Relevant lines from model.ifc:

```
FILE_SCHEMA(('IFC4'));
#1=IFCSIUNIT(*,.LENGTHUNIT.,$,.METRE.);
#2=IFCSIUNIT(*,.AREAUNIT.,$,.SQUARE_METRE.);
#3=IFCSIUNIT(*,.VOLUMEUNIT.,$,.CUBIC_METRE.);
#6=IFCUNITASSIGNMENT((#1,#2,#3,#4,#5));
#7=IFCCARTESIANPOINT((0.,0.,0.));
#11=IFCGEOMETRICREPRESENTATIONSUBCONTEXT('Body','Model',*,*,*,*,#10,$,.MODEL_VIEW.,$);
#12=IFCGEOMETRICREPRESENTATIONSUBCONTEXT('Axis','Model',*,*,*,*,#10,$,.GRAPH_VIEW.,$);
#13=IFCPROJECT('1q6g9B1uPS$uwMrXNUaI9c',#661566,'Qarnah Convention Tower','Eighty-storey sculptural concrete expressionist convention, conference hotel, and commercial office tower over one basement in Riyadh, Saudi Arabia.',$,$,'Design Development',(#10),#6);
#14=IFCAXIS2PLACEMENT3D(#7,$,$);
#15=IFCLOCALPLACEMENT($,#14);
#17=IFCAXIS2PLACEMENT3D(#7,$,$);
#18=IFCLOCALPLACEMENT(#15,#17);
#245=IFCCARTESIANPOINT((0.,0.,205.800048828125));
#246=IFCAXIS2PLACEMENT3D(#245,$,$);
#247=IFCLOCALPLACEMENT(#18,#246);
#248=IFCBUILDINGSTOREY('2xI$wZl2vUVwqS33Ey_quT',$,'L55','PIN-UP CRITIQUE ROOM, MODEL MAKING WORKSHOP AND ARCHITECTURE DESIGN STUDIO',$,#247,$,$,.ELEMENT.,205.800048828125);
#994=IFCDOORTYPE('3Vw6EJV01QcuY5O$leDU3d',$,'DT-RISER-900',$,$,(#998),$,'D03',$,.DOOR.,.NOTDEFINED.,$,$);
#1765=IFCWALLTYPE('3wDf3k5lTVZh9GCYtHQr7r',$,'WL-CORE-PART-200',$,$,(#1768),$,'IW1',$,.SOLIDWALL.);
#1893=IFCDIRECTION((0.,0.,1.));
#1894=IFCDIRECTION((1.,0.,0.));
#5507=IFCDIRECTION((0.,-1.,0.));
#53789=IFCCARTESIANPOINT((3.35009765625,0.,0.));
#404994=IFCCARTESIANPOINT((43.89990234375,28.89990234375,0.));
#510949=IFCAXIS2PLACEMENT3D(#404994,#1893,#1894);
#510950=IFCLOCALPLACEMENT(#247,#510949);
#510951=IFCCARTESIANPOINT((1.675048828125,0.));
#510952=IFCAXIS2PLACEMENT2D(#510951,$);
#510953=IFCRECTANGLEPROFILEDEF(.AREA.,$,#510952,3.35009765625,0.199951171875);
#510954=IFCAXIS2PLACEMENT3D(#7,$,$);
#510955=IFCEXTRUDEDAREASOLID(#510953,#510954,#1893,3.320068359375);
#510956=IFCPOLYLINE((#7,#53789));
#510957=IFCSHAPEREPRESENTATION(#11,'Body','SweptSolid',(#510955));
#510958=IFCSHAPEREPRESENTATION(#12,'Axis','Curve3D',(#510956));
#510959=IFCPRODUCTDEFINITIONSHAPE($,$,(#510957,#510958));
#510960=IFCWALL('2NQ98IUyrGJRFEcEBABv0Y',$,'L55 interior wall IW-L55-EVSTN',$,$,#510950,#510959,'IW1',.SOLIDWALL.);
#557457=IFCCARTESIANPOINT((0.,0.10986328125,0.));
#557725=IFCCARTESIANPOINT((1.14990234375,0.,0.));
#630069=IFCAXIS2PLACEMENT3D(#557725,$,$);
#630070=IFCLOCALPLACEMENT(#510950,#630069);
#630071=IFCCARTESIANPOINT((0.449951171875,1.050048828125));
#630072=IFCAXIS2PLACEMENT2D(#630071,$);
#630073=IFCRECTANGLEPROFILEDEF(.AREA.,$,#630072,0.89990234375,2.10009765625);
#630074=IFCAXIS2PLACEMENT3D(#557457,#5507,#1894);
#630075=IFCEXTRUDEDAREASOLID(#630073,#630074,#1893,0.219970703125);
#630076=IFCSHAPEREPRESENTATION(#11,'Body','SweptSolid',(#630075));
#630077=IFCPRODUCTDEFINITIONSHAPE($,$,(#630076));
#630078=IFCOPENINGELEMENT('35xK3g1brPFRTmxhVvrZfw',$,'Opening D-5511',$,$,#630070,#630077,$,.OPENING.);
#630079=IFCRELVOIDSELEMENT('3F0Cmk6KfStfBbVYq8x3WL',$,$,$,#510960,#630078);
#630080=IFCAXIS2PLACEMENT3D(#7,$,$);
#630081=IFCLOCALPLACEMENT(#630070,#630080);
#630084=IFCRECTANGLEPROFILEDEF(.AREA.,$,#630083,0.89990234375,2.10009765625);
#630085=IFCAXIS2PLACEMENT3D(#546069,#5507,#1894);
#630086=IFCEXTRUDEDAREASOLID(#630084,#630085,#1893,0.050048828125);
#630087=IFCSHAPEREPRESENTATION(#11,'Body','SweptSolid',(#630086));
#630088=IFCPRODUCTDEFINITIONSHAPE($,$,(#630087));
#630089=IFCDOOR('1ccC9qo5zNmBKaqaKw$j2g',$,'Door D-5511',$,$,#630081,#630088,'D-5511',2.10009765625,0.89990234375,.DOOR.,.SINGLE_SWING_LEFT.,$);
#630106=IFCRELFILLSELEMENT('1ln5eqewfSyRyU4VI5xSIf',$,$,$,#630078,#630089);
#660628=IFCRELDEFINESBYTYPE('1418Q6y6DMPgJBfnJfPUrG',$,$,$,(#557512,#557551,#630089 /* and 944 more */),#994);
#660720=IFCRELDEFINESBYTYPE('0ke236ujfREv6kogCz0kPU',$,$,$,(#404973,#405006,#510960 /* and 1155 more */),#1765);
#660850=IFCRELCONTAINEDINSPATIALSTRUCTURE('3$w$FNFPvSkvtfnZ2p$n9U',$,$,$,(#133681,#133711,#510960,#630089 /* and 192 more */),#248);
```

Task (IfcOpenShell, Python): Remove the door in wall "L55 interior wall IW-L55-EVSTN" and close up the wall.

```python
import ifcopenshell
import ifcopenshell.api.feature
import ifcopenshell.api.root
import ifcopenshell.geom
import ifcopenshell.util.shape

model = ifcopenshell.open("model.ifc")
settings = ifcopenshell.geom.settings()


def volume(element):
    """Net volume in cubic metres, openings subtracted."""
    shape = ifcopenshell.geom.create_shape(settings, element)
    return ifcopenshell.util.shape.get_volume(shape.geometry)


door = model.by_guid("1ccC9qo5zNmBKaqaKw$j2g")
opening = door.FillsVoids[0].RelatingOpeningElement
wall = opening.VoidsElements[0].RelatingBuildingElement
before = volume(wall)

ifcopenshell.api.root.remove_product(model, product=door)
ifcopenshell.api.feature.remove_feature(model, feature=opening)

after = volume(wall)

print(f"wall volume {before:.3f} -> {after:.3f} m3")

model.write("model_edited.ifc")
```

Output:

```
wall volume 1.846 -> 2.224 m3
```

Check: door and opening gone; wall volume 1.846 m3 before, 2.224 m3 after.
